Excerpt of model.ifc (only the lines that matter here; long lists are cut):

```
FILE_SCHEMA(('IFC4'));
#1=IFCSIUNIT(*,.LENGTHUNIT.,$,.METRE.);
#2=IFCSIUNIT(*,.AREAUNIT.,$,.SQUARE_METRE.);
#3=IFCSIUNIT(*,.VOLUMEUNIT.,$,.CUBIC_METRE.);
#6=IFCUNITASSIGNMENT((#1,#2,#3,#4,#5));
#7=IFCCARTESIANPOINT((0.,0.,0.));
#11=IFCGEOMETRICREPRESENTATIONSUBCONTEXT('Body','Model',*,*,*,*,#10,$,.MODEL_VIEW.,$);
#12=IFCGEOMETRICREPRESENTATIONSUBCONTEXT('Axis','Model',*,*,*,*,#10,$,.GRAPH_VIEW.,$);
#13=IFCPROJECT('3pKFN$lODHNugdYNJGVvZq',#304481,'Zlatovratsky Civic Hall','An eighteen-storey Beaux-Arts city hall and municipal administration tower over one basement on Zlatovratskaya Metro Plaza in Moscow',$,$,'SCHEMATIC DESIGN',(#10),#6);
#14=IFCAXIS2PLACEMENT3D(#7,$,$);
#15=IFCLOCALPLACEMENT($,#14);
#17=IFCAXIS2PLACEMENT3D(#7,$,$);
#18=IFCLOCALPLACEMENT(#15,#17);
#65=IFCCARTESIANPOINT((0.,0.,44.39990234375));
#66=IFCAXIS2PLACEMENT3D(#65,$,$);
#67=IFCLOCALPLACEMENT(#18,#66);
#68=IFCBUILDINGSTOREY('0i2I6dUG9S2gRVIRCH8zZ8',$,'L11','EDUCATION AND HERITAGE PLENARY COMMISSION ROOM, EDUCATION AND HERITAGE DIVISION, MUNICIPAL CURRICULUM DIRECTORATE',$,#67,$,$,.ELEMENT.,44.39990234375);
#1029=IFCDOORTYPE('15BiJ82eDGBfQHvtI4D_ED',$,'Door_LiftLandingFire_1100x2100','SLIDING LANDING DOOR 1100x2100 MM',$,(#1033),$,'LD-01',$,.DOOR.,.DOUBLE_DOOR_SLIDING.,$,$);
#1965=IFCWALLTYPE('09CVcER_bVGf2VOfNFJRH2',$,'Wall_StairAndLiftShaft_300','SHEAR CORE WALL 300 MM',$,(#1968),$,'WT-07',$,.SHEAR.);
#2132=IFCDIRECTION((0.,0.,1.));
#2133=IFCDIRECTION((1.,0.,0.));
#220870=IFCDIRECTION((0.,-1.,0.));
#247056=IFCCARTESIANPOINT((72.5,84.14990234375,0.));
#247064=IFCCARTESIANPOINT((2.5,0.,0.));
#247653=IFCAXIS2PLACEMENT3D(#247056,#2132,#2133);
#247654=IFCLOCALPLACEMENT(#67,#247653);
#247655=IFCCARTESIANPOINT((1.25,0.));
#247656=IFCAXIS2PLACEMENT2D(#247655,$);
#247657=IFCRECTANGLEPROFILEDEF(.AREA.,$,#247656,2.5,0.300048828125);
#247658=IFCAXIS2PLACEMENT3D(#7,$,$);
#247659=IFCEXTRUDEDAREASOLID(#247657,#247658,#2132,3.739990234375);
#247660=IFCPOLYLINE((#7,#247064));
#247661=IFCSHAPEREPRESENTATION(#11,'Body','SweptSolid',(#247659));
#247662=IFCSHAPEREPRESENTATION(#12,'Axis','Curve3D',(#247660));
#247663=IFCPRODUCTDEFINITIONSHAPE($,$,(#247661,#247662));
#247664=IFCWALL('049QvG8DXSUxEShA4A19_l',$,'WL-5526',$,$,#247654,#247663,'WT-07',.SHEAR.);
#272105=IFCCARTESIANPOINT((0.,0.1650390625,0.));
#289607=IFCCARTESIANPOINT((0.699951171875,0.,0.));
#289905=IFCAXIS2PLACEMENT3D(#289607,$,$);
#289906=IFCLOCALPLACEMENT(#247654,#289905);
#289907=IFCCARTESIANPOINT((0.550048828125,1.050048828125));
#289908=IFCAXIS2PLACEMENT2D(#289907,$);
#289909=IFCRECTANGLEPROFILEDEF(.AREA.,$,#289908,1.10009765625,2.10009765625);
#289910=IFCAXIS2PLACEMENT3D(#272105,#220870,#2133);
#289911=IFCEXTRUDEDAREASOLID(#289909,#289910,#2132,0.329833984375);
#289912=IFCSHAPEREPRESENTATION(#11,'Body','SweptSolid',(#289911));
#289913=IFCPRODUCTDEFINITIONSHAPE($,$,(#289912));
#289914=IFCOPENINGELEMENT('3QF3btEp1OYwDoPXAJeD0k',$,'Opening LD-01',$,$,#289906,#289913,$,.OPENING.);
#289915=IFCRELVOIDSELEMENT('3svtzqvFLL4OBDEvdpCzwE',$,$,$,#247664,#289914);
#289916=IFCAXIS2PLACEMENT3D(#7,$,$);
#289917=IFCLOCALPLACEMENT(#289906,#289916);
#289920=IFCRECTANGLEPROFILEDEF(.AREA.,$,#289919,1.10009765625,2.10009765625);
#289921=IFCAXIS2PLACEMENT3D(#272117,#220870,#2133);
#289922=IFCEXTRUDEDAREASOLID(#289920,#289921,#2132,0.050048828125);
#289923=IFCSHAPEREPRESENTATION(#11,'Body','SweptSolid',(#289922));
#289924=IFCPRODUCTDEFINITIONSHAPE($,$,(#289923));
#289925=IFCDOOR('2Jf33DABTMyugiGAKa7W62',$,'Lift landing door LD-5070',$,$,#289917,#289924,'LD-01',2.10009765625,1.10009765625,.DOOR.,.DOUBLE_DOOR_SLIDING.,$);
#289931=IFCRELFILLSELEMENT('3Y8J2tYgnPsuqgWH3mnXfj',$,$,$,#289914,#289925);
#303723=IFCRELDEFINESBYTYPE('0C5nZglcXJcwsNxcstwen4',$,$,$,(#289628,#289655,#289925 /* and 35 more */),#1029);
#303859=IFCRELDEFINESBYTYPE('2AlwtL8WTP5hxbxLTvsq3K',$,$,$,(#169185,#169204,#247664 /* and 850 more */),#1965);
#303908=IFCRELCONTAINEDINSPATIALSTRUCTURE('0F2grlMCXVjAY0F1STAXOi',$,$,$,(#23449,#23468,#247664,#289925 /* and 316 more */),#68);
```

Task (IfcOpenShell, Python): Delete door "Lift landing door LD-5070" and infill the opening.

```python
import ifcopenshell
import ifcopenshell.api.feature
import ifcopenshell.api.root
import ifcopenshell.geom
import ifcopenshell.util.shape

model = ifcopenshell.open("model.ifc")
settings = ifcopenshell.geom.settings()


def volume(element):
    """Net volume in cubic metres, openings subtracted."""
    shape = ifcopenshell.geom.create_shape(settings, element)
    return ifcopenshell.util.shape.get_volume(shape.geometry)


door = model.by_guid("2Jf33DABTMyugiGAKa7W62")
opening = door.FillsVoids[0].RelatingOpeningElement
wall = opening.VoidsElements[0].RelatingBuildingElement
before = volume(wall)

ifcopenshell.api.root.remove_product(model, product=door)
ifcopenshell.api.feature.remove_feature(model, feature=opening)

after = volume(wall)

print(f"wall volume {before:.3f} -> {after:.3f} m3")

model.write("model-out.ifc")
```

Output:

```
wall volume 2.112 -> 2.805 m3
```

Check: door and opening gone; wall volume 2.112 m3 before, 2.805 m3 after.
